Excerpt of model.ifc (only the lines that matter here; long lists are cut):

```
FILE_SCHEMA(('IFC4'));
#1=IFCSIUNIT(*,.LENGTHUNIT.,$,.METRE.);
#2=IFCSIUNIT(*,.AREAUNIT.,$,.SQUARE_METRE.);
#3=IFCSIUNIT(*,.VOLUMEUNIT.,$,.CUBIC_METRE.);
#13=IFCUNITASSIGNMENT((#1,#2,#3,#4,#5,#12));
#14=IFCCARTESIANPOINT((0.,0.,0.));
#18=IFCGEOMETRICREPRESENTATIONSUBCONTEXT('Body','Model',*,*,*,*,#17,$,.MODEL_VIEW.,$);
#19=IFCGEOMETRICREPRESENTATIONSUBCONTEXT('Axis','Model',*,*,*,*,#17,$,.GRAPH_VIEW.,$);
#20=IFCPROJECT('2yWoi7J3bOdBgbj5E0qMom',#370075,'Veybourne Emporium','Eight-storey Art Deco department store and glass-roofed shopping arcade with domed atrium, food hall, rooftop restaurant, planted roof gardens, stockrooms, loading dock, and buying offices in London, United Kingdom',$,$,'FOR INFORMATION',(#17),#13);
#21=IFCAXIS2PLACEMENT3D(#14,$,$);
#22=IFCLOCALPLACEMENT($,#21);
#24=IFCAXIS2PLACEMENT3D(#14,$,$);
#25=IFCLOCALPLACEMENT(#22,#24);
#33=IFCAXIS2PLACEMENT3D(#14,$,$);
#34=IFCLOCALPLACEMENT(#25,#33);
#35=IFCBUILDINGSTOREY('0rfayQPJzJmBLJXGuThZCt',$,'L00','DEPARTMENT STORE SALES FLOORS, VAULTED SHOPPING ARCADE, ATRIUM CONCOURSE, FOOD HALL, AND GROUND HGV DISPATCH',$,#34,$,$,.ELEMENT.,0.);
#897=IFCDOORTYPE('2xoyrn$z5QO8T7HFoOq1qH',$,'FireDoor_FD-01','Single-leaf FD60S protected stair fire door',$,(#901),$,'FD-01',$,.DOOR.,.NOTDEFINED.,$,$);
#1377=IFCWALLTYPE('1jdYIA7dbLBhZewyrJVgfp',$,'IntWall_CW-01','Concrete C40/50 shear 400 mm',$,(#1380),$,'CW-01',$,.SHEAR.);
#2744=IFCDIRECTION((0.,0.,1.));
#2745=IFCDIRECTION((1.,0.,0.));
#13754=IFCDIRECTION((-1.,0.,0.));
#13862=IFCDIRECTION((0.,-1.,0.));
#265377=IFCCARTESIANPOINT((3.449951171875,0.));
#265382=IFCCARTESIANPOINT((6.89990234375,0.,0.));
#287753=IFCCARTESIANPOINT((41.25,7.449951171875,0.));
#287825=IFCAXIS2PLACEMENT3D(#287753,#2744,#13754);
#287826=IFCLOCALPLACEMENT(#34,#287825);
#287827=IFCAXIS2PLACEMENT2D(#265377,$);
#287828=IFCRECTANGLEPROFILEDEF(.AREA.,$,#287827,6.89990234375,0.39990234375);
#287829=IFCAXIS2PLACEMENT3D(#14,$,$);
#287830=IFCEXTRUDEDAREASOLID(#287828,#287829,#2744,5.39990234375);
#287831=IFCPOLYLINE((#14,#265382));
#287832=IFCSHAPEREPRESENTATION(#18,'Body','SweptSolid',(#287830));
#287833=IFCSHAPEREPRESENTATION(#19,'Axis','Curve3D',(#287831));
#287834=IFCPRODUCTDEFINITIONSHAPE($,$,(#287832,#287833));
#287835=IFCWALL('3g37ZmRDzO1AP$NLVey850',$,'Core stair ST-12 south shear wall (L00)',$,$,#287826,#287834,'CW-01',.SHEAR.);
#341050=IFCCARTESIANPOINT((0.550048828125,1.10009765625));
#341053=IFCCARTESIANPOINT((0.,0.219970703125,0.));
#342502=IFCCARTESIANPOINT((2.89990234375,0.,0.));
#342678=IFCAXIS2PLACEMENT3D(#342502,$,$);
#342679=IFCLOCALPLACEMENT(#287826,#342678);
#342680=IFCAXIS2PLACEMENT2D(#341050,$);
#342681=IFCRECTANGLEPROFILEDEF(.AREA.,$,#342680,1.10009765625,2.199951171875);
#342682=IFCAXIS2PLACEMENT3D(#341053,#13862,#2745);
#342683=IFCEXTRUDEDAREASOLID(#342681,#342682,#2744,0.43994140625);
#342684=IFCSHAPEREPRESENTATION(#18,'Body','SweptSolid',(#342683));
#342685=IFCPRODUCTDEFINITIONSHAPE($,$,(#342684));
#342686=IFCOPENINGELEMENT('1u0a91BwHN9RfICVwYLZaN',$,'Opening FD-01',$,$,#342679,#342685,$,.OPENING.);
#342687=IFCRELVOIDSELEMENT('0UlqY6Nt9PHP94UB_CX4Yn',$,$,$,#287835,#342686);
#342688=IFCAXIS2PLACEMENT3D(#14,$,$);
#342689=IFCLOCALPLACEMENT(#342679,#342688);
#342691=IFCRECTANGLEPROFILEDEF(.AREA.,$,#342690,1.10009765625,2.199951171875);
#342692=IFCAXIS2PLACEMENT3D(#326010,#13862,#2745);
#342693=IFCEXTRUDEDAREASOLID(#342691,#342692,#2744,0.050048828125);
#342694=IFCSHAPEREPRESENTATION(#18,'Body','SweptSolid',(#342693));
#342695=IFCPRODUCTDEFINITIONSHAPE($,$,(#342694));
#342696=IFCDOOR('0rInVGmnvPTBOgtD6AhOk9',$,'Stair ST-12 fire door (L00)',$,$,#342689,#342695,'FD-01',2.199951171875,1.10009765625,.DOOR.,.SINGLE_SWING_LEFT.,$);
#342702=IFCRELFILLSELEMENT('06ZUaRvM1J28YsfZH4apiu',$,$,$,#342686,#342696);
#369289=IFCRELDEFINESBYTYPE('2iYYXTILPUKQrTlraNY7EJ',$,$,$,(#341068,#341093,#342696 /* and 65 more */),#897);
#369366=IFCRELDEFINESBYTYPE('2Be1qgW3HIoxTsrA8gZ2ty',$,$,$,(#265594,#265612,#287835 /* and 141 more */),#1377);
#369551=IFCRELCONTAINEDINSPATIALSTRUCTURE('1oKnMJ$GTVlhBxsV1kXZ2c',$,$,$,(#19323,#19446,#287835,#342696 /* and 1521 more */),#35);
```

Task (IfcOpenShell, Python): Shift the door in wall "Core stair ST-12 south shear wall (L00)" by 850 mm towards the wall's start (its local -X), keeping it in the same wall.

```python
import ifcopenshell
import ifcopenshell.api.geometry
import ifcopenshell.util.placement

model = ifcopenshell.open("model.ifc")

door = model.by_guid("0rInVGmnvPTBOgtD6AhOk9")
opening = door.FillsVoids[0].RelatingOpeningElement
wall = opening.VoidsElements[0].RelatingBuildingElement

wall_matrix = ifcopenshell.util.placement.get_local_placement(wall.ObjectPlacement)
shift = wall_matrix[:3, 0] * -0.85
before = ifcopenshell.util.placement.get_local_placement(door.ObjectPlacement)[:3, 3].copy()

# The door is placed relative to its opening, so it follows when the opening moves.
matrix = ifcopenshell.util.placement.get_local_placement(opening.ObjectPlacement)
matrix[:3, 3] += shift
ifcopenshell.api.geometry.edit_object_placement(
    model, product=opening, matrix=matrix, is_si=False, should_transform_children=True
)

after = ifcopenshell.util.placement.get_local_placement(door.ObjectPlacement)[:3, 3]
print("door moved by", (after - before).round(3) + 0.0)

model.write("model_updated.ifc")
```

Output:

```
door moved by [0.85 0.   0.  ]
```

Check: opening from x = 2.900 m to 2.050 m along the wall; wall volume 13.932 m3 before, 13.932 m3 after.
